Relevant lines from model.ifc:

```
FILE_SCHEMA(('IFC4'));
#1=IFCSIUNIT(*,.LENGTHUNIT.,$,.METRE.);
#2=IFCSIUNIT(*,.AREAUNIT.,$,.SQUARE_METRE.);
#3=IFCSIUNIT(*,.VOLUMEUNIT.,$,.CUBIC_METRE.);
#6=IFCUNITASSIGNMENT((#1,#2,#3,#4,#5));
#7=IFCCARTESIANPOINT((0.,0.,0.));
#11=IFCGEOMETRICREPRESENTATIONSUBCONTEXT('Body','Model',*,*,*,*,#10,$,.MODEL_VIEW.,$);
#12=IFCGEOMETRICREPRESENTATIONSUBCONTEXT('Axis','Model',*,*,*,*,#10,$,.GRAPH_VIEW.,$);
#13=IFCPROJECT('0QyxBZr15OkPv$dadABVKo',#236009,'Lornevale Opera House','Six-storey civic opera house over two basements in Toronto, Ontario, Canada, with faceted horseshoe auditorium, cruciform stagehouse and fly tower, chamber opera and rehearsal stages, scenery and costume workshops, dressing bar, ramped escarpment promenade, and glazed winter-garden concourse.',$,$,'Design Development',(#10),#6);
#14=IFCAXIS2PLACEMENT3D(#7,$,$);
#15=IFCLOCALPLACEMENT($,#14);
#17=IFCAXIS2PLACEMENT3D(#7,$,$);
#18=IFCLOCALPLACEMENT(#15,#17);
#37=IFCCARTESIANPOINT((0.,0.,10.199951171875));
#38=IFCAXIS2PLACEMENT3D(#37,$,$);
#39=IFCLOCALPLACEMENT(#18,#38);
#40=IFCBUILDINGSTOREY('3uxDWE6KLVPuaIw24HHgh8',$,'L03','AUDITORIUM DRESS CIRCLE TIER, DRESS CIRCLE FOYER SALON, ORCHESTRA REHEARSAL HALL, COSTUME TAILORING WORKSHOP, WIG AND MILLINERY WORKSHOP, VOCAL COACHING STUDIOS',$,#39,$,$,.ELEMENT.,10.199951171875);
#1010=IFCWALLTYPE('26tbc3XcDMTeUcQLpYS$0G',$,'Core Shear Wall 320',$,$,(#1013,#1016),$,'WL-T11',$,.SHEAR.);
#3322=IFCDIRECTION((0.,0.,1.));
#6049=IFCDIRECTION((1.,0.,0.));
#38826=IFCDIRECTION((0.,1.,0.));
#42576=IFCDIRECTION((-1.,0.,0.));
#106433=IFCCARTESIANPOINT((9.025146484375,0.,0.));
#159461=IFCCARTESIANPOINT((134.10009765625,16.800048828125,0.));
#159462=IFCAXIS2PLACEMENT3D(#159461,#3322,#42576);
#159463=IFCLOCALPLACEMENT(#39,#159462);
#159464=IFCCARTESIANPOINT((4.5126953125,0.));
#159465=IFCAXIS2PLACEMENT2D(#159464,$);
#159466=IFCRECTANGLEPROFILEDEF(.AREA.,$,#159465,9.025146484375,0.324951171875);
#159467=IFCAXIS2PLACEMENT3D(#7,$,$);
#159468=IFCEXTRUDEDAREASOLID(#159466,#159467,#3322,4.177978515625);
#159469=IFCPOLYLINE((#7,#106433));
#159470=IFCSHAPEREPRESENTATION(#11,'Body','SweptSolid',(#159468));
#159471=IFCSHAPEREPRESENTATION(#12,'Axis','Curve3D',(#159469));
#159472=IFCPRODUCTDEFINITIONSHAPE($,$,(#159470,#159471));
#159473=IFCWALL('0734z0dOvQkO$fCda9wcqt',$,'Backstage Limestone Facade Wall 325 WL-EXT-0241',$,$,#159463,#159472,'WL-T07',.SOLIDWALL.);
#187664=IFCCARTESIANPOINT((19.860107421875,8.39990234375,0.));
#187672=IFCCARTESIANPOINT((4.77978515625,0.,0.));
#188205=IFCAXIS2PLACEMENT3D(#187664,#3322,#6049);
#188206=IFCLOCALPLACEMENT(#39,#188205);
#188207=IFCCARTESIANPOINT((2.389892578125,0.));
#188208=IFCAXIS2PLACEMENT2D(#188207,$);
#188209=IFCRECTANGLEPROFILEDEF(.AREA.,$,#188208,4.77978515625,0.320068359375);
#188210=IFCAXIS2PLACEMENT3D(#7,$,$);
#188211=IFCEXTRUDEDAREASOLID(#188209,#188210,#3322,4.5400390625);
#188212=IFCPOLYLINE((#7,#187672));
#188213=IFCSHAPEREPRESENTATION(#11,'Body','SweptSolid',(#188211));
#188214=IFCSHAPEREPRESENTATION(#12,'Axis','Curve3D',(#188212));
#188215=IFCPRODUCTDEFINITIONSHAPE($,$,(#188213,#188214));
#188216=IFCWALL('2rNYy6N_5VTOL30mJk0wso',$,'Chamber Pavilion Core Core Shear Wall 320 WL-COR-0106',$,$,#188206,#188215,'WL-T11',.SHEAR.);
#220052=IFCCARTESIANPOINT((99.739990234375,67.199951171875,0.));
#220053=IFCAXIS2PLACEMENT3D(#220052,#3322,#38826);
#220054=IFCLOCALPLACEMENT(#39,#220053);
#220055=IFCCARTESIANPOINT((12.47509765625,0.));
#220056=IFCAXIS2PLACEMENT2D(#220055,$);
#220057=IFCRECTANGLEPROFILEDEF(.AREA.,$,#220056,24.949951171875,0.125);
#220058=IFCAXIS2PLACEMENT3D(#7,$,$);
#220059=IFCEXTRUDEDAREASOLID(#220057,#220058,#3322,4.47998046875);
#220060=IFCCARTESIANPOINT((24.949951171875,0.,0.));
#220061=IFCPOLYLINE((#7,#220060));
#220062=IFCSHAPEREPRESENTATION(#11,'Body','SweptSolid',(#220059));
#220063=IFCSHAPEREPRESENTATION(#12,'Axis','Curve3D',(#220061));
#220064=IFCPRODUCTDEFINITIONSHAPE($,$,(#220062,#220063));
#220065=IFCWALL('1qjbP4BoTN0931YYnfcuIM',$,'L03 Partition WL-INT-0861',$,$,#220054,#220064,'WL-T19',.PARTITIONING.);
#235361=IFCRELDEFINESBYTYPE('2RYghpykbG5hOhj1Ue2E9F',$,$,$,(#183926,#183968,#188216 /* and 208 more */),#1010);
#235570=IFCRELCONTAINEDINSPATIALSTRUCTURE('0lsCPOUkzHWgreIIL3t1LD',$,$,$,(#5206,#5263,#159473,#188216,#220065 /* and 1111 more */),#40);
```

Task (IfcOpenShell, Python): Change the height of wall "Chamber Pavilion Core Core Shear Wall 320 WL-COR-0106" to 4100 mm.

```python
import ifcopenshell
import ifcopenshell.geom
import ifcopenshell.util.representation
import ifcopenshell.util.shape
import ifcopenshell.util.unit

model = ifcopenshell.open("model.ifc")
unit_scale = ifcopenshell.util.unit.calculate_unit_scale(model)
settings = ifcopenshell.geom.settings()


def volume(element):
    """Net volume in cubic metres, openings subtracted."""
    shape = ifcopenshell.geom.create_shape(settings, element)
    return ifcopenshell.util.shape.get_volume(shape.geometry)


wall = model.by_guid("2rNYy6N_5VTOL30mJk0wso")
before = volume(wall)

body = ifcopenshell.util.representation.get_representation(wall, "Model", "Body")
solid = body.Items[0]
old_height = solid.Depth
solid.Depth = 4.1 / unit_scale
after = volume(wall)

print(f"height {old_height:g} -> {solid.Depth:g}, volume {before:.3f} -> {after:.3f} m3")

model.write("model_edited.ifc")
```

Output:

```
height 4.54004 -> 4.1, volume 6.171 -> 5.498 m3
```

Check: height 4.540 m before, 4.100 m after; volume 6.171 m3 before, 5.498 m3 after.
